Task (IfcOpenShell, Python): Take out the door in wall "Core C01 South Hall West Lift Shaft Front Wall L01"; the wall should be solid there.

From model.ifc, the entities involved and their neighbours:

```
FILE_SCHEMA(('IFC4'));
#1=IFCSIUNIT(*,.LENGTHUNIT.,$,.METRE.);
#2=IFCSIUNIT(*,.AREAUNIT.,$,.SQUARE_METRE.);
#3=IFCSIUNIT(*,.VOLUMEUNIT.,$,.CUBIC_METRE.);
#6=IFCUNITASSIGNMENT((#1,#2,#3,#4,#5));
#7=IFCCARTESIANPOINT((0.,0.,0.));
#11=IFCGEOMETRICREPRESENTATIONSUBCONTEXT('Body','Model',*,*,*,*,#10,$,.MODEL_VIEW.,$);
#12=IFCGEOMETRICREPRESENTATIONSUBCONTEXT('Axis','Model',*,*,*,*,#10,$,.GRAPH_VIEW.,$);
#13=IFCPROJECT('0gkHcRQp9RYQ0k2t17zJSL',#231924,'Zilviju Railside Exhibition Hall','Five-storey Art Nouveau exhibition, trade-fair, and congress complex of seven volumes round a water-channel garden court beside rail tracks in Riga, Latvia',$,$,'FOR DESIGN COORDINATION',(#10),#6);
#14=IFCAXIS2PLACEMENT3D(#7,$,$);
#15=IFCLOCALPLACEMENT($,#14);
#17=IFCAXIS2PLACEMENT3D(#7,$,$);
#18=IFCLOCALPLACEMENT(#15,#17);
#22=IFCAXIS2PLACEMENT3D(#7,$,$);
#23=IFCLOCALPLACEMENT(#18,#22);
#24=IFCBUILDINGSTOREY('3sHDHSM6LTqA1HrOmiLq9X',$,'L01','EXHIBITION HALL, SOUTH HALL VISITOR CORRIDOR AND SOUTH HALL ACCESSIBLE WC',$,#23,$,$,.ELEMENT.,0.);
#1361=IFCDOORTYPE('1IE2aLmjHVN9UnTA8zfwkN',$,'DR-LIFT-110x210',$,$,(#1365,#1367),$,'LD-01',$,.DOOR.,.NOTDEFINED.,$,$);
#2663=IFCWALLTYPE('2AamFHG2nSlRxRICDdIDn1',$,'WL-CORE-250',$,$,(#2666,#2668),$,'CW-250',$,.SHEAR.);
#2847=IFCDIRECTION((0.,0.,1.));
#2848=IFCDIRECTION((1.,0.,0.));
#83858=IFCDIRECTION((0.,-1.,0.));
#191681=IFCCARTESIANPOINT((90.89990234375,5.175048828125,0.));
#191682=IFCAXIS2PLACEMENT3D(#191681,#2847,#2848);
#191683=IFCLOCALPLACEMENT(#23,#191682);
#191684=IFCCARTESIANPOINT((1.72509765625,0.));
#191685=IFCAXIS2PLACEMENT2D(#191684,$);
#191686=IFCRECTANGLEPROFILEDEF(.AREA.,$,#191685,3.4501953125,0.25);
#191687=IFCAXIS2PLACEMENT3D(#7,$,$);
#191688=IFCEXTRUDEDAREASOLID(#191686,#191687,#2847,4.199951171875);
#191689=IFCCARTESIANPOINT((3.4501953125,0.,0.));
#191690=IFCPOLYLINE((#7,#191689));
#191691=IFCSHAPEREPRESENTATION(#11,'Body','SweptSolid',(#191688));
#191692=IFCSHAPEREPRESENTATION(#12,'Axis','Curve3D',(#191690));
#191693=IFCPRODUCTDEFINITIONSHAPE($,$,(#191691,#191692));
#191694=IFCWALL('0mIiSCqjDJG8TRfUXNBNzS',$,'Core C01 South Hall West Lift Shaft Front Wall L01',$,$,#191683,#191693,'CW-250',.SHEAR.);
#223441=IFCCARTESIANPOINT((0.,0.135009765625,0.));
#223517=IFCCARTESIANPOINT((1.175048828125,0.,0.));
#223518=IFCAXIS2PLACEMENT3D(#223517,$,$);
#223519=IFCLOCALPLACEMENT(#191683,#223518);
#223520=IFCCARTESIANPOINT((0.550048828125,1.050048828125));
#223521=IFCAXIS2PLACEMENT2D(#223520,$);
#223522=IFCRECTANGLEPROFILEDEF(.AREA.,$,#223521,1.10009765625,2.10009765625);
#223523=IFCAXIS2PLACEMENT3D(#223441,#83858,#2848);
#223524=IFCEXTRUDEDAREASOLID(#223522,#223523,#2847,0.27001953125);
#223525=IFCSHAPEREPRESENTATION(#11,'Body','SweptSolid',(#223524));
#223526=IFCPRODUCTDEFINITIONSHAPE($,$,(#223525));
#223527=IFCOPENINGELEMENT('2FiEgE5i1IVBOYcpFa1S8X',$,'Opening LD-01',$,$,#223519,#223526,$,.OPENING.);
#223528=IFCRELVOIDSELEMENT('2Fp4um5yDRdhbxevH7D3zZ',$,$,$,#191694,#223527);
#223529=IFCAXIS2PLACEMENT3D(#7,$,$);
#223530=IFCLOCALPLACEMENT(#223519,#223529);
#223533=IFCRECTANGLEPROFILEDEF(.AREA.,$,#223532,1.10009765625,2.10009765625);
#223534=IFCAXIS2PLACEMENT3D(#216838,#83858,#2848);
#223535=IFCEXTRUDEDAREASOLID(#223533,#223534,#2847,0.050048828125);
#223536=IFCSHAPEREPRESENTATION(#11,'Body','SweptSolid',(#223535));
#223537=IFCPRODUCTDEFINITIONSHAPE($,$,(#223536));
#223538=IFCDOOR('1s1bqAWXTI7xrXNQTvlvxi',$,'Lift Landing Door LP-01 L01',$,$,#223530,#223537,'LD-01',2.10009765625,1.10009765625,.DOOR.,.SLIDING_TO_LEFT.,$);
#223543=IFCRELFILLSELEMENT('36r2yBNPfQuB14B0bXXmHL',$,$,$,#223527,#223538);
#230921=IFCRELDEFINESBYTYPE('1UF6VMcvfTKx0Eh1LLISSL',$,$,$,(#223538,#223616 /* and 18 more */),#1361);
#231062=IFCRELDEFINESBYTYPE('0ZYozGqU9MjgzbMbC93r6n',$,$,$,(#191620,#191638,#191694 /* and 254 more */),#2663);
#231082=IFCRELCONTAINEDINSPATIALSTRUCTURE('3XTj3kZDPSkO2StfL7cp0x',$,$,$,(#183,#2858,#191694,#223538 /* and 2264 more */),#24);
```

```python
import ifcopenshell
import ifcopenshell.api.feature
import ifcopenshell.api.root
import ifcopenshell.geom
import ifcopenshell.util.shape

model = ifcopenshell.open("model.ifc")
settings = ifcopenshell.geom.settings()


def volume(element):
    """Net volume in cubic metres, openings subtracted."""
    shape = ifcopenshell.geom.create_shape(settings, element)
    return ifcopenshell.util.shape.get_volume(shape.geometry)


door = model.by_guid("1s1bqAWXTI7xrXNQTvlvxi")
opening = door.FillsVoids[0].RelatingOpeningElement
wall = opening.VoidsElements[0].RelatingBuildingElement
before = volume(wall)

ifcopenshell.api.root.remove_product(model, product=door)
ifcopenshell.api.feature.remove_feature(model, feature=opening)

after = volume(wall)

print(f"wall volume {before:.3f} -> {after:.3f} m3")

model.write("model_updated.ifc")
```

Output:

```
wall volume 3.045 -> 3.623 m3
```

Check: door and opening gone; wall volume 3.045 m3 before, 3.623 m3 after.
